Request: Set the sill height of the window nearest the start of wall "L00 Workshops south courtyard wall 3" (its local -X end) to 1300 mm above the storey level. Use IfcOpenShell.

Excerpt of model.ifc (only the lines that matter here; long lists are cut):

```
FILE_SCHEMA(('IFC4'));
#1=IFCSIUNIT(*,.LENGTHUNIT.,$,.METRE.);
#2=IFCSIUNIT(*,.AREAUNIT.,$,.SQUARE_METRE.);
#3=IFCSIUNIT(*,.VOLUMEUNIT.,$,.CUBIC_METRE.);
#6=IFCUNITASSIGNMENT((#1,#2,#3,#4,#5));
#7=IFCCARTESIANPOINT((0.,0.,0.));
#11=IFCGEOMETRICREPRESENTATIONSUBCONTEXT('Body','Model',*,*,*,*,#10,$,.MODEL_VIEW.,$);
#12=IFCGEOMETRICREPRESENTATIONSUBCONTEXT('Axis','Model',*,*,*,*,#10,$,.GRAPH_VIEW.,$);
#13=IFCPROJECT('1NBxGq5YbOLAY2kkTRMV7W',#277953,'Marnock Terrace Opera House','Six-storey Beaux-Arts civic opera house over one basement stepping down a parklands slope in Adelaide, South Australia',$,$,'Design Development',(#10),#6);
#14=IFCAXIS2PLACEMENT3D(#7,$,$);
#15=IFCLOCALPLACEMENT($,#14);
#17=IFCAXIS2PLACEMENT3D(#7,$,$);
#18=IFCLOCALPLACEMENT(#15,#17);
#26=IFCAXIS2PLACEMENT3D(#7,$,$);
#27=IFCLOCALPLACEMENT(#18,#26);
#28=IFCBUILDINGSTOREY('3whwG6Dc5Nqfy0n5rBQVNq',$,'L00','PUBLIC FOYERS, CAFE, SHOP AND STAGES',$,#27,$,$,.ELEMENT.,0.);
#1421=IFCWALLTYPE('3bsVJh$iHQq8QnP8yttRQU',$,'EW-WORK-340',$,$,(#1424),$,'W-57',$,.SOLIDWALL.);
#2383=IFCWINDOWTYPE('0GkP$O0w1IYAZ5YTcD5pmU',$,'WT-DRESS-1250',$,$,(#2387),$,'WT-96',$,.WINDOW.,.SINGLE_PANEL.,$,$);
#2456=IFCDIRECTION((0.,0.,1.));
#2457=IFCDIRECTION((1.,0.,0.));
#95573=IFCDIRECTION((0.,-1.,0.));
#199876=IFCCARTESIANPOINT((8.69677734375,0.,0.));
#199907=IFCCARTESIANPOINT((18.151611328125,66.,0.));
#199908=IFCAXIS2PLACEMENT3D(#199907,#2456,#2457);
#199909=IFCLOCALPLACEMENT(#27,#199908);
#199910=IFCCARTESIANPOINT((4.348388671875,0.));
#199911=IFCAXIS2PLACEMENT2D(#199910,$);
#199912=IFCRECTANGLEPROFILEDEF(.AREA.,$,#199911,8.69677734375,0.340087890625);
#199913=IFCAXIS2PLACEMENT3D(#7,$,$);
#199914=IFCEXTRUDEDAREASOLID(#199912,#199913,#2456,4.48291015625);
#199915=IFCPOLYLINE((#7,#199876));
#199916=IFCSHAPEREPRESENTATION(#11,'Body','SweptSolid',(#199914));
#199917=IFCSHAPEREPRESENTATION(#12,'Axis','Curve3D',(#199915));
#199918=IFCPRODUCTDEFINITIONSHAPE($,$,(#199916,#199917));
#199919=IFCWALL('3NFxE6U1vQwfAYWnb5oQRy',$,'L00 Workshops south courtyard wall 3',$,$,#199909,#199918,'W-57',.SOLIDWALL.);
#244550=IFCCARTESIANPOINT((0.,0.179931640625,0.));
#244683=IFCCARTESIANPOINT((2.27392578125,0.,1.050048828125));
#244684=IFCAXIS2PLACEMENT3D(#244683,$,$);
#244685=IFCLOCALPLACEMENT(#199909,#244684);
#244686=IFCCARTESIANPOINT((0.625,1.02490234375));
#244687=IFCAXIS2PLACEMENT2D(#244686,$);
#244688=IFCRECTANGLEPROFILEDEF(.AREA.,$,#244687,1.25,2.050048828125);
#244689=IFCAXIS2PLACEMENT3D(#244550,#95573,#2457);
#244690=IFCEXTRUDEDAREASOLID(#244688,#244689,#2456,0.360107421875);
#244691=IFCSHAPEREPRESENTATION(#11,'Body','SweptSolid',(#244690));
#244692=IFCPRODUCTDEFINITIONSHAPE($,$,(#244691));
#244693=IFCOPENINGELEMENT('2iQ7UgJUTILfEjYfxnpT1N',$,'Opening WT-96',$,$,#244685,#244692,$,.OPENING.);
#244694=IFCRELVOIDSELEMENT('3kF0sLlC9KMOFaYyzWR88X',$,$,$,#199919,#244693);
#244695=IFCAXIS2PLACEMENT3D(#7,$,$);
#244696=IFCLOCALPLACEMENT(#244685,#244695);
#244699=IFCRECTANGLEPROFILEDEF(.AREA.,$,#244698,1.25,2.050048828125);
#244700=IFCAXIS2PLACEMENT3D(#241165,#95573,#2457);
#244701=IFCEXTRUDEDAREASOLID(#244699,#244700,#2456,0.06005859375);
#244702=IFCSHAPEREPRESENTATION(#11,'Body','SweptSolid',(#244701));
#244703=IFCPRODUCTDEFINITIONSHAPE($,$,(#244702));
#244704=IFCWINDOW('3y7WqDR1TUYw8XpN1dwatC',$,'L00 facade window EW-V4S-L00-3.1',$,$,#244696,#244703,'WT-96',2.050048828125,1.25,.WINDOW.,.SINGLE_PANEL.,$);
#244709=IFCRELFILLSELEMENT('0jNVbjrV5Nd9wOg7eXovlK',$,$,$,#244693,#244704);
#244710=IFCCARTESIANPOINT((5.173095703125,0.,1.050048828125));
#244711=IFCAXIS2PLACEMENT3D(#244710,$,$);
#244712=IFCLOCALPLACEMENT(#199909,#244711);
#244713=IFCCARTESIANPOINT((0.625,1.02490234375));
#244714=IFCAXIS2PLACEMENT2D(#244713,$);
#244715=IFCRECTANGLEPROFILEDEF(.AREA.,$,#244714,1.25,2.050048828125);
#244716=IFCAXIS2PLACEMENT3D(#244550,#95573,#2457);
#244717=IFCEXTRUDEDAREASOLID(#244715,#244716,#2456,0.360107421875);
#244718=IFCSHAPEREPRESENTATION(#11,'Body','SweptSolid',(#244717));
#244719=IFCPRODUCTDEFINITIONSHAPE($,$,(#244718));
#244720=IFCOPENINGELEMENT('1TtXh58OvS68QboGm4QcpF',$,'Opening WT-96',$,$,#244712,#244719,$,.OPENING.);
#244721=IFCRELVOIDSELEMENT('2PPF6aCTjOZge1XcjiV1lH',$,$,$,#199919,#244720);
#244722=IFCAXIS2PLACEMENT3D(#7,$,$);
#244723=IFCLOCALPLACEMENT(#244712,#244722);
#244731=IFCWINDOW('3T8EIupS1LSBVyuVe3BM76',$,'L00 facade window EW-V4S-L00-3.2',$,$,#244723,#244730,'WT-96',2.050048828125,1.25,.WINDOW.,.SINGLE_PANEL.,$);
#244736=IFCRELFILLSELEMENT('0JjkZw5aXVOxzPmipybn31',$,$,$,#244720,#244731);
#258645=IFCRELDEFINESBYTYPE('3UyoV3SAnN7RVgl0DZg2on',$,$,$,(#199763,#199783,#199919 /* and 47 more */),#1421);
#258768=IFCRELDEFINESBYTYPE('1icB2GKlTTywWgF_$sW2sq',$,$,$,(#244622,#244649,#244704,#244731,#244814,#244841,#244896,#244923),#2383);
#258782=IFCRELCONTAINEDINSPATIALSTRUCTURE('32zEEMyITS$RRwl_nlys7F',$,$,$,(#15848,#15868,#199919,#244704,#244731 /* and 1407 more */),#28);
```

```python
import numpy as np
import ifcopenshell
import ifcopenshell.api.geometry
import ifcopenshell.geom
import ifcopenshell.util.element
import ifcopenshell.util.placement
import ifcopenshell.util.shape
import ifcopenshell.util.unit

model = ifcopenshell.open("model.ifc")
unit_scale = ifcopenshell.util.unit.calculate_unit_scale(model)

window = model.by_guid("3y7WqDR1TUYw8XpN1dwatC")
opening = window.FillsVoids[0].RelatingOpeningElement
storey = ifcopenshell.util.element.get_container(window, ifc_class="IfcBuildingStorey")
level = ifcopenshell.util.placement.get_local_placement(storey.ObjectPlacement)[2, 3]

# The opening's origin need not be at the sill, so measure its lowest point.
shape = ifcopenshell.geom.create_shape(ifcopenshell.geom.settings(), opening)
bottom = ifcopenshell.util.shape.get_shape_bottom_elevation(shape, shape.geometry) / unit_scale
dz = level + 1.3 / unit_scale - bottom

shift = np.array([0.0, 0.0, dz])
# The window is placed relative to its opening, so it follows when the opening moves.
matrix = ifcopenshell.util.placement.get_local_placement(opening.ObjectPlacement)
matrix[:3, 3] += shift
ifcopenshell.api.geometry.edit_object_placement(
    model, product=opening, matrix=matrix, is_si=False, should_transform_children=True
)

print(f"moved by {dz * unit_scale:+.3f} m")

model.write("model-out.ifc")
```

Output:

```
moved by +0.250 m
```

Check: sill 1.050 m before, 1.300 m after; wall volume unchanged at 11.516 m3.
